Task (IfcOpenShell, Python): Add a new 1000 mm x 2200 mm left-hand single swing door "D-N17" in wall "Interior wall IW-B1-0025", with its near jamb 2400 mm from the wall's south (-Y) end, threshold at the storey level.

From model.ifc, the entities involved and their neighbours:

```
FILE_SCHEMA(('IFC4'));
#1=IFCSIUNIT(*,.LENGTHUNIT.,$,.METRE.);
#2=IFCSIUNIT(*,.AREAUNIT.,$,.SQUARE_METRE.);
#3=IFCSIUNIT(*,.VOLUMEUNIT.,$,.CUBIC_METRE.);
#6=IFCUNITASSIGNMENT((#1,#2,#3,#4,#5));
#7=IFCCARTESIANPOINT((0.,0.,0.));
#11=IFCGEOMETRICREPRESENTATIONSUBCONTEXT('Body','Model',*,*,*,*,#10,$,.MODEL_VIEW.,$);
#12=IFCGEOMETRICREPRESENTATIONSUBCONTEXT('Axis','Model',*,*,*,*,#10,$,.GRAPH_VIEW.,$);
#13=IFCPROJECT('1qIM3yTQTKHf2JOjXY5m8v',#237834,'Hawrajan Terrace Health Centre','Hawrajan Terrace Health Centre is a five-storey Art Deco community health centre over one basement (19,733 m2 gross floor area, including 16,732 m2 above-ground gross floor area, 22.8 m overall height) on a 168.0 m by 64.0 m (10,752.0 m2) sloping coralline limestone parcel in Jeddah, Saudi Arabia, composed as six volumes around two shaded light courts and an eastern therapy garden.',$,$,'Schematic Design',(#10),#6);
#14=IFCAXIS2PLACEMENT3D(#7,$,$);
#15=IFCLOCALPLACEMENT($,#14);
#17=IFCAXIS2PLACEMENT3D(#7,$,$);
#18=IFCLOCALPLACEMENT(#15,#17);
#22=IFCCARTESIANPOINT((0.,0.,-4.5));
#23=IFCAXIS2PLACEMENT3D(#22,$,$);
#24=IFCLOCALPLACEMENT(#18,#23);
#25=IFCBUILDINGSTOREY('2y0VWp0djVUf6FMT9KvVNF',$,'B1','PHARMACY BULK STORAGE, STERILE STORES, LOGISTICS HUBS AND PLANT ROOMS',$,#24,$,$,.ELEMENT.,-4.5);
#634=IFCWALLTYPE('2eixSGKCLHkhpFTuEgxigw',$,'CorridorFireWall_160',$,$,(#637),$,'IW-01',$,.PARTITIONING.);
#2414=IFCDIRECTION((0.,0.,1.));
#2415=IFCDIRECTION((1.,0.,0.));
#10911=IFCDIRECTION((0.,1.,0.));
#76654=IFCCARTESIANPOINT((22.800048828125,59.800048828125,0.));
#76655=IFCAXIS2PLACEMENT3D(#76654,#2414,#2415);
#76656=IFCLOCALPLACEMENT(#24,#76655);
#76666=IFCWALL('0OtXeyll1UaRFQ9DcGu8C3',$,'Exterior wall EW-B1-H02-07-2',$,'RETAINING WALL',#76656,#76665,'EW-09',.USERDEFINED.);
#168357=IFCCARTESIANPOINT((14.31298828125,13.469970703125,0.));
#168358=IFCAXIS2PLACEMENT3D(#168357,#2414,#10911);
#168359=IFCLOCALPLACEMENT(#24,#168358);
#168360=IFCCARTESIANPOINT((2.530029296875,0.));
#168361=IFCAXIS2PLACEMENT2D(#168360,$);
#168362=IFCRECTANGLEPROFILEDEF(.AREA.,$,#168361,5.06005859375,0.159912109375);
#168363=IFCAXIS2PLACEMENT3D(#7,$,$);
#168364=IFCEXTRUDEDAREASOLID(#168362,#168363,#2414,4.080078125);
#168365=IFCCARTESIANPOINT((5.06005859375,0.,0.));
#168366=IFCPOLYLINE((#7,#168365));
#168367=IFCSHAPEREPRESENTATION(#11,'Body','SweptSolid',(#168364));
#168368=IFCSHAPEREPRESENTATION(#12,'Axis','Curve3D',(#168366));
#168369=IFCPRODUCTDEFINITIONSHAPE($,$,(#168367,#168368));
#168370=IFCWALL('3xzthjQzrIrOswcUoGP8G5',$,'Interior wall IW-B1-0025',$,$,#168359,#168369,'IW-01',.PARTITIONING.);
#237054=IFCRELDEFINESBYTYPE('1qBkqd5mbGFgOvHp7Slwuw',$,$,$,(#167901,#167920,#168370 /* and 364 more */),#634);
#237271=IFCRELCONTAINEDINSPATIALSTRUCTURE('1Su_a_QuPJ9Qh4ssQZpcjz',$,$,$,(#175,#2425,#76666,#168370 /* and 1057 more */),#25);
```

```python
import numpy as np
import ifcopenshell
import ifcopenshell.api.feature
import ifcopenshell.api.geometry
import ifcopenshell.api.root
import ifcopenshell.api.spatial
import ifcopenshell.geom
import ifcopenshell.util.element
import ifcopenshell.util.placement
import ifcopenshell.util.representation
import ifcopenshell.util.shape
import ifcopenshell.util.unit

model = ifcopenshell.open("model.ifc")
unit_scale = ifcopenshell.util.unit.calculate_unit_scale(model)
settings = ifcopenshell.geom.settings()


def volume(element):
    """Net volume in cubic metres, openings subtracted."""
    shape = ifcopenshell.geom.create_shape(settings, element)
    return ifcopenshell.util.shape.get_volume(shape.geometry)


wall = model.by_guid("3xzthjQzrIrOswcUoGP8G5")
storey = ifcopenshell.util.element.get_container(wall, ifc_class="IfcBuildingStorey")
context = ifcopenshell.util.representation.get_context(model, "Model", "Body", "MODEL_VIEW")
before = volume(wall)

width, height, from_end, sill = 1, 2.2, 2.4, 0.0  # metres

# The wall runs along its own X axis, and the end named is its -X end.
wall_shape = ifcopenshell.geom.create_shape(settings, wall)
x, y, z = ifcopenshell.util.shape.get_vertices(wall_shape.geometry).T
start = x.min() + from_end
face, thickness = float(y.min()), float(y.max() - y.min())
wall_matrix = ifcopenshell.util.placement.get_local_placement(wall.ObjectPlacement)
level = ifcopenshell.util.placement.get_local_placement(storey.ObjectPlacement)[2, 3]


def in_wall(x, y):
    """Placement at x, y metres in the wall's axes, at sill height."""
    matrix = wall_matrix.copy()
    matrix[:, 3] = wall_matrix @ np.array([x / unit_scale, y / unit_scale, 0.0, 1.0])
    matrix[2, 3] = level + sill / unit_scale
    return matrix


# Opening: a box that overshoots both wall faces by 50 mm.
opening = ifcopenshell.api.root.create_entity(model, ifc_class="IfcOpeningElement", predefined_type="OPENING")
box = ifcopenshell.api.geometry.add_wall_representation(
    model, context=context, length=width, height=height, thickness=thickness + 0.1
)
ifcopenshell.api.geometry.assign_representation(model, product=opening, representation=box)
ifcopenshell.api.geometry.edit_object_placement(model, product=opening, matrix=in_wall(start, face - 0.05), is_si=False)
ifcopenshell.api.feature.add_feature(model, feature=opening, element=wall)

door = ifcopenshell.api.root.create_entity(model, ifc_class="IfcDoor", name="D-N17", predefined_type="DOOR")
door.OverallWidth, door.OverallHeight = width / unit_scale, height / unit_scale
door.OperationType = "SINGLE_SWING_LEFT"
body = ifcopenshell.api.geometry.add_door_representation(
    model,
    context=context,
    overall_width=door.OverallWidth,
    overall_height=door.OverallHeight,
    operation_type="SINGLE_SWING_LEFT",
    lining_properties={"LiningDepth": thickness / unit_scale, "ThresholdDepth": thickness / unit_scale},
)
ifcopenshell.api.geometry.assign_representation(model, product=door, representation=body)
ifcopenshell.api.spatial.assign_container(model, products=[door], relating_structure=storey)
ifcopenshell.api.feature.add_filling(model, opening=opening, element=door)

# The lining spans the wall, so the door starts at the wall face.
ifcopenshell.api.geometry.edit_object_placement(model, product=door, matrix=in_wall(start, face), is_si=False)

after = volume(wall)

print(f"wall volume {before:.3f} -> {after:.3f} m3")

model.write("model_edited.ifc")
```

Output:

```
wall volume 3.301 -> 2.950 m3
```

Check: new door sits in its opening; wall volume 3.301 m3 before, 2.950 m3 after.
